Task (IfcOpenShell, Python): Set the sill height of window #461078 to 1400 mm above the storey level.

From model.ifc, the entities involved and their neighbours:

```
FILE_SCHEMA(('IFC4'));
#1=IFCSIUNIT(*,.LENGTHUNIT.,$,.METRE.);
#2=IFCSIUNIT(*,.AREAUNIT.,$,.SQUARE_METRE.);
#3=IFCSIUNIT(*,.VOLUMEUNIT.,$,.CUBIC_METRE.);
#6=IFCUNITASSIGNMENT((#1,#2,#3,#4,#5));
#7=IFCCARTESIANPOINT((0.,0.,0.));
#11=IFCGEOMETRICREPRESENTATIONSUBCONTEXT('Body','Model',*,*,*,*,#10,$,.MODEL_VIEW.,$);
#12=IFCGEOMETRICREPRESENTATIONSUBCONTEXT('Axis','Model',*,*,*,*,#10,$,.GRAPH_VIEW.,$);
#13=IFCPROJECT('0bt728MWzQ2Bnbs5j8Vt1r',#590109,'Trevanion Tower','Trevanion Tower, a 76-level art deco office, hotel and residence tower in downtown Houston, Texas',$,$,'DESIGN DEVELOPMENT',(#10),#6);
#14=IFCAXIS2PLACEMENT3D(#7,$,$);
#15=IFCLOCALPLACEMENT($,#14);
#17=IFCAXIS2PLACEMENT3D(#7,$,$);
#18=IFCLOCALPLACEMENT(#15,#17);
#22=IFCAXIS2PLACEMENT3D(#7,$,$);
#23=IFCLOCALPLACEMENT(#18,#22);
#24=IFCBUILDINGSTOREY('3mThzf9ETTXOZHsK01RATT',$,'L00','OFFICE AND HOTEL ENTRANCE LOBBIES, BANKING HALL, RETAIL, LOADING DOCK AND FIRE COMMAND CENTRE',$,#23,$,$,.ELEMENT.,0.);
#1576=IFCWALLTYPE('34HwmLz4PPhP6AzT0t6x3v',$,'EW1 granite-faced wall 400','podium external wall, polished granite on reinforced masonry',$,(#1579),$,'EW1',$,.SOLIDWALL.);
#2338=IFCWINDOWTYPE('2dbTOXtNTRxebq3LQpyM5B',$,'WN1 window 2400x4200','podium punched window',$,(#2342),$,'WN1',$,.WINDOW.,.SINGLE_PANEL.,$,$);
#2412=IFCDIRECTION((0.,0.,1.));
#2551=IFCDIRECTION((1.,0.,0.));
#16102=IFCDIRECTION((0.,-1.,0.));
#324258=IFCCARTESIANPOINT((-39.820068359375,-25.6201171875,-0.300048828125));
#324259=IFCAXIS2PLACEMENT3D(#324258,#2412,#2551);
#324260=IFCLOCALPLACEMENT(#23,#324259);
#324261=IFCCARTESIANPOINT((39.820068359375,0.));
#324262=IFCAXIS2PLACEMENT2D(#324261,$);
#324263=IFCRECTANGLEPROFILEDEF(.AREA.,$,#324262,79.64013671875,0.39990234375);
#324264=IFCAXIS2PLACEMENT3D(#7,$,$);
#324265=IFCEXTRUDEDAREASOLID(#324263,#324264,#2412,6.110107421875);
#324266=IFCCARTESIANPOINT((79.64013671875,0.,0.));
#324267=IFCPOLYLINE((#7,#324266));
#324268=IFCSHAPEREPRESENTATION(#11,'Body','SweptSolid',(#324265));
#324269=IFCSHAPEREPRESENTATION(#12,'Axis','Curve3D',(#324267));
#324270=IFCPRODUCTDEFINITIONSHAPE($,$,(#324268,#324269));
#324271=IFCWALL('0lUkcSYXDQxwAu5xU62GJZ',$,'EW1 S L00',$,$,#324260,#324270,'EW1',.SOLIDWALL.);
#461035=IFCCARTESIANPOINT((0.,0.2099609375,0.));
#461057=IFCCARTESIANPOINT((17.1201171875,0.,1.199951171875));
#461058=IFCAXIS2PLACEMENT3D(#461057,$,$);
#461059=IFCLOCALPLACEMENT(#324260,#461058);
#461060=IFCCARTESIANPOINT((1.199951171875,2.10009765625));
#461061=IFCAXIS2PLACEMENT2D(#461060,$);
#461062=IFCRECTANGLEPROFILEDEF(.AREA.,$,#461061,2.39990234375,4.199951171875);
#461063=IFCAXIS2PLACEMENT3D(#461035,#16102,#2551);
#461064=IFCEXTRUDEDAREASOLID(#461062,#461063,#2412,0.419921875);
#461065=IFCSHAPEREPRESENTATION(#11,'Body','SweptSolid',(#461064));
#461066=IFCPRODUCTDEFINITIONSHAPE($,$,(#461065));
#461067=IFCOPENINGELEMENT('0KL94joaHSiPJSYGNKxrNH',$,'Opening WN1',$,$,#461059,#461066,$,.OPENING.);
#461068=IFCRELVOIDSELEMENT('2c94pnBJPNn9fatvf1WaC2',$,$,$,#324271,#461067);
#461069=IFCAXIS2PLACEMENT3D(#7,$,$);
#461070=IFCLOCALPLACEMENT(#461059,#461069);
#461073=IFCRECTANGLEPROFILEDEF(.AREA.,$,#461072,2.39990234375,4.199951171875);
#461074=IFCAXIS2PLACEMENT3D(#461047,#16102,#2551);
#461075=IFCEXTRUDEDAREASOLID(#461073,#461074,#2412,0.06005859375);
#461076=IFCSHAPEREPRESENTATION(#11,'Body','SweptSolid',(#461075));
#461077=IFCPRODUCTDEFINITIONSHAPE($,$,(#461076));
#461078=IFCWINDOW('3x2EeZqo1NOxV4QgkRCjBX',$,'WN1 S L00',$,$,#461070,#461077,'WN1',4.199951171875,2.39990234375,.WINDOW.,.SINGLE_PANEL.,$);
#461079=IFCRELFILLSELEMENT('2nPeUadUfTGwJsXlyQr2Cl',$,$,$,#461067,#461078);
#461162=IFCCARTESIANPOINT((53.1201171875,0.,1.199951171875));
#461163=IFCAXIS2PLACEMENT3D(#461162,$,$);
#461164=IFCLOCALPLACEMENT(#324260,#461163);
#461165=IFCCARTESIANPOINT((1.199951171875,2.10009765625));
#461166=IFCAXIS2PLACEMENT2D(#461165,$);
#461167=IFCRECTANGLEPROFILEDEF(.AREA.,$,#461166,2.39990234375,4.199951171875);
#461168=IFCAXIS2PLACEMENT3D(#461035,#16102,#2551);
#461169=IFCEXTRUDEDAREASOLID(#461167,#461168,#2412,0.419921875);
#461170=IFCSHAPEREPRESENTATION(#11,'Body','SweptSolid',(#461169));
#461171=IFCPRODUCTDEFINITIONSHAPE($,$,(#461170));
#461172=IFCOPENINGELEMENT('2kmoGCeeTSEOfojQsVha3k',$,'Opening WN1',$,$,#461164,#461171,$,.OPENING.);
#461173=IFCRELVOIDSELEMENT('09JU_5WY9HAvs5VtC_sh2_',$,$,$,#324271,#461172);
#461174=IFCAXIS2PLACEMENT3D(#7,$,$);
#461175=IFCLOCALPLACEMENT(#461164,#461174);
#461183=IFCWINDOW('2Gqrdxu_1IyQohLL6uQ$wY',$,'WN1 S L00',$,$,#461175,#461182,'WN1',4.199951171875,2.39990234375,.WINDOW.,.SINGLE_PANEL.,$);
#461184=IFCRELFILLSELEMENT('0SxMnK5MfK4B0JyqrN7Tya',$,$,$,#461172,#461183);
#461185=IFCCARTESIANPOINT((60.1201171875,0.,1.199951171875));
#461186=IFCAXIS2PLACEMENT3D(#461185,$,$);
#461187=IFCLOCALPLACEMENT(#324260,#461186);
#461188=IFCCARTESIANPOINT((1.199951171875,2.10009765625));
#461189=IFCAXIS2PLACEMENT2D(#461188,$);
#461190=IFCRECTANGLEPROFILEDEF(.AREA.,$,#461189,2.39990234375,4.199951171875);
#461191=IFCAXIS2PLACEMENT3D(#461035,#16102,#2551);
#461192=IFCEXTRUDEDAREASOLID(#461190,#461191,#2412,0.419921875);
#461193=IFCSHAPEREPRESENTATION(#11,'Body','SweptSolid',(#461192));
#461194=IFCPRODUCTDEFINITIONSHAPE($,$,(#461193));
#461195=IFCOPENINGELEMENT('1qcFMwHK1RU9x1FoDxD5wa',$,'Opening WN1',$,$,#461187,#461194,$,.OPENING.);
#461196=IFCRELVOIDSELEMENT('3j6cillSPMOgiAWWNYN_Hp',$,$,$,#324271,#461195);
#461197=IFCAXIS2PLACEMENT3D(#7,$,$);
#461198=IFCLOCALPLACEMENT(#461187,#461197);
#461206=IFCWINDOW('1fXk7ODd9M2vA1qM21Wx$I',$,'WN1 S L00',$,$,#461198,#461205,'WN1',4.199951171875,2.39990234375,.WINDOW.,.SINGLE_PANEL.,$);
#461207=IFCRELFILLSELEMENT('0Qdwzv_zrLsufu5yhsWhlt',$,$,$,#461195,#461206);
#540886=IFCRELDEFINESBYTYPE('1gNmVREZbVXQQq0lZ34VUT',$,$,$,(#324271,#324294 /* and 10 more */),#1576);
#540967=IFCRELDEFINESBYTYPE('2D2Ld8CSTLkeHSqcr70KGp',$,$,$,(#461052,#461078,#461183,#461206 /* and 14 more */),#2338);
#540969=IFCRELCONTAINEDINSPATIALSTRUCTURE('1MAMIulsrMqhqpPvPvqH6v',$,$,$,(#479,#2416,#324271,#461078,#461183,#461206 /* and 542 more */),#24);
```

```python
import numpy as np
import ifcopenshell
import ifcopenshell.api.geometry
import ifcopenshell.geom
import ifcopenshell.util.element
import ifcopenshell.util.placement
import ifcopenshell.util.shape
import ifcopenshell.util.unit

model = ifcopenshell.open("model.ifc")
unit_scale = ifcopenshell.util.unit.calculate_unit_scale(model)

window = model.by_guid("3x2EeZqo1NOxV4QgkRCjBX")
opening = window.FillsVoids[0].RelatingOpeningElement
storey = ifcopenshell.util.element.get_container(window, ifc_class="IfcBuildingStorey")
level = ifcopenshell.util.placement.get_local_placement(storey.ObjectPlacement)[2, 3]

# The opening's origin need not be at the sill, so measure its lowest point.
shape = ifcopenshell.geom.create_shape(ifcopenshell.geom.settings(), opening)
bottom = ifcopenshell.util.shape.get_shape_bottom_elevation(shape, shape.geometry) / unit_scale
dz = level + 1.4 / unit_scale - bottom

shift = np.array([0.0, 0.0, dz])
# The window is placed relative to its opening, so it follows when the opening moves.
matrix = ifcopenshell.util.placement.get_local_placement(opening.ObjectPlacement)
matrix[:3, 3] += shift
ifcopenshell.api.geometry.edit_object_placement(
    model, product=opening, matrix=matrix, is_si=False, should_transform_children=True
)

print(f"moved by {dz * unit_scale:+.3f} m")

model.write("model_edited.ifc")
```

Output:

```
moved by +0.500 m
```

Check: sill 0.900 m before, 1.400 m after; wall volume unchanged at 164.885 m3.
